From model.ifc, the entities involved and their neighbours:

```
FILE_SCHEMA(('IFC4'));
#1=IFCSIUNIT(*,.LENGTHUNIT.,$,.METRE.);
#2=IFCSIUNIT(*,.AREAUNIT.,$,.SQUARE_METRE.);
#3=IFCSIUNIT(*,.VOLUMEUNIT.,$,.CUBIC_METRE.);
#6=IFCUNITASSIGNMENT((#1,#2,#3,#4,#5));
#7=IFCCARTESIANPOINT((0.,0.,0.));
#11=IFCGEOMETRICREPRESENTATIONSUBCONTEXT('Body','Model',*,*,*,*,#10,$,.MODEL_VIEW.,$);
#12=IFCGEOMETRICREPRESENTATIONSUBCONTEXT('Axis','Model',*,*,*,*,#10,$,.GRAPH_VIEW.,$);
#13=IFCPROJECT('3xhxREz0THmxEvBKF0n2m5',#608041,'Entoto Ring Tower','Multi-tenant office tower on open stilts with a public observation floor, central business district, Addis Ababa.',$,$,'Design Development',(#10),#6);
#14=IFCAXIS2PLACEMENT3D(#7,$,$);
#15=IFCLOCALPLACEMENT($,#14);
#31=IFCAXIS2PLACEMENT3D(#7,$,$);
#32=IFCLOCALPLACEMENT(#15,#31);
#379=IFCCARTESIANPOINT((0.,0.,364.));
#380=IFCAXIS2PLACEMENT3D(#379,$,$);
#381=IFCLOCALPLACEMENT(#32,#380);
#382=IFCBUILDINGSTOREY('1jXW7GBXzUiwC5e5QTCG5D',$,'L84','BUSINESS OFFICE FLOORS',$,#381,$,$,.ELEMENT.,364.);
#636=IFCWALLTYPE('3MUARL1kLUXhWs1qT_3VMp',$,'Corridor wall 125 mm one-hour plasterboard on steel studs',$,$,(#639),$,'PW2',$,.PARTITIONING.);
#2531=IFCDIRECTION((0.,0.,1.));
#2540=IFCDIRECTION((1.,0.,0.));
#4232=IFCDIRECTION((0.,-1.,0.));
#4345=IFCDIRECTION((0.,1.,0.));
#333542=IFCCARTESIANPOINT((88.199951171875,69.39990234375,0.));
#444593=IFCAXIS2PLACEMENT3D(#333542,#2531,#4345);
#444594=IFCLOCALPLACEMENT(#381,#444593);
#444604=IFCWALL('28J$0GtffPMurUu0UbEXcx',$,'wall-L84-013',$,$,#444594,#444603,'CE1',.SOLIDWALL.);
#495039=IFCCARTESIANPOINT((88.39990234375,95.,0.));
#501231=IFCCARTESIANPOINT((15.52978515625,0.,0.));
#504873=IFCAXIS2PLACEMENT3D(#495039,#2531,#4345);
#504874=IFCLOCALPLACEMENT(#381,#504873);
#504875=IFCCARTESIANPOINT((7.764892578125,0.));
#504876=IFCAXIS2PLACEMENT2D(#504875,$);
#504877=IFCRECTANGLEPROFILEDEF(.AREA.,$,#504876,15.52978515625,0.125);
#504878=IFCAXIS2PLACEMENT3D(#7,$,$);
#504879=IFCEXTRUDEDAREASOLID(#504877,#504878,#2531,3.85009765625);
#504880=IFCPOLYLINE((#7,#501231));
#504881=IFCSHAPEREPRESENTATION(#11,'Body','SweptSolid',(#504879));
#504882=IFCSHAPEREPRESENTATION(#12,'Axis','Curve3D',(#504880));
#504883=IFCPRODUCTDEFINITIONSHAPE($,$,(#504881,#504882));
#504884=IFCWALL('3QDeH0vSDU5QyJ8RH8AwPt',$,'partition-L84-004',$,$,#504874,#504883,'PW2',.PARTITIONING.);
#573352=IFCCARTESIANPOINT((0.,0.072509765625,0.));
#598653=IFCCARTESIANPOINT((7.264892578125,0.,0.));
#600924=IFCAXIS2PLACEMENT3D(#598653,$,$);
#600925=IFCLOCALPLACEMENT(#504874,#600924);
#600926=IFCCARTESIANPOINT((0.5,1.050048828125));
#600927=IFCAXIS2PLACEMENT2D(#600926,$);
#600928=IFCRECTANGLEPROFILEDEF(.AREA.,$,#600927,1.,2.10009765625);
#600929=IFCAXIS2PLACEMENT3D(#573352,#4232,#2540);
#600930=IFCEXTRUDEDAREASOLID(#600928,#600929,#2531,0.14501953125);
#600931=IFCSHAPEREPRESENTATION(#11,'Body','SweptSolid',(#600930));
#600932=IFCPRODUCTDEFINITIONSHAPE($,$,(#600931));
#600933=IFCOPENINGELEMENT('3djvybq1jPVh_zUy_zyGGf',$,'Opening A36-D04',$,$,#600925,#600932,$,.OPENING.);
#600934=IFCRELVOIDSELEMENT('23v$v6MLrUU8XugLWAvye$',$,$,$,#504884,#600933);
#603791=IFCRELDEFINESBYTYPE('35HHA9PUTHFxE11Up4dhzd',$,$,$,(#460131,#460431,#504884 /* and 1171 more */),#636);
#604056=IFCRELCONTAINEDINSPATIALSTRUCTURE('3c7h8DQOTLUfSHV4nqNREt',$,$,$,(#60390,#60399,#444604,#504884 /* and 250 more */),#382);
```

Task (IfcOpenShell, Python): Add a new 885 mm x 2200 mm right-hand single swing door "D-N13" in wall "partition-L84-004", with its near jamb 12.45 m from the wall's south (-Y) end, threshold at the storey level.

```python
import numpy as np
import ifcopenshell
import ifcopenshell.api.feature
import ifcopenshell.api.geometry
import ifcopenshell.api.root
import ifcopenshell.api.spatial
import ifcopenshell.geom
import ifcopenshell.util.element
import ifcopenshell.util.placement
import ifcopenshell.util.representation
import ifcopenshell.util.shape
import ifcopenshell.util.unit

model = ifcopenshell.open("model.ifc")
unit_scale = ifcopenshell.util.unit.calculate_unit_scale(model)
settings = ifcopenshell.geom.settings()


def volume(element):
    """Net volume in cubic metres, openings subtracted."""
    shape = ifcopenshell.geom.create_shape(settings, element)
    return ifcopenshell.util.shape.get_volume(shape.geometry)


wall = model.by_guid("3QDeH0vSDU5QyJ8RH8AwPt")
storey = ifcopenshell.util.element.get_container(wall, ifc_class="IfcBuildingStorey")
context = ifcopenshell.util.representation.get_context(model, "Model", "Body", "MODEL_VIEW")
before = volume(wall)

width, height, from_end, sill = 0.885, 2.2, 12.45, 0.0  # metres

# The wall runs along its own X axis, and the end named is its -X end.
wall_shape = ifcopenshell.geom.create_shape(settings, wall)
x, y, z = ifcopenshell.util.shape.get_vertices(wall_shape.geometry).T
start = x.min() + from_end
face, thickness = float(y.min()), float(y.max() - y.min())
wall_matrix = ifcopenshell.util.placement.get_local_placement(wall.ObjectPlacement)
level = ifcopenshell.util.placement.get_local_placement(storey.ObjectPlacement)[2, 3]


def in_wall(x, y):
    """Placement at x, y metres in the wall's axes, at sill height."""
    matrix = wall_matrix.copy()
    matrix[:, 3] = wall_matrix @ np.array([x / unit_scale, y / unit_scale, 0.0, 1.0])
    matrix[2, 3] = level + sill / unit_scale
    return matrix


# Opening: a box that overshoots both wall faces by 50 mm.
opening = ifcopenshell.api.root.create_entity(model, ifc_class="IfcOpeningElement", predefined_type="OPENING")
box = ifcopenshell.api.geometry.add_wall_representation(
    model, context=context, length=width, height=height, thickness=thickness + 0.1
)
ifcopenshell.api.geometry.assign_representation(model, product=opening, representation=box)
ifcopenshell.api.geometry.edit_object_placement(model, product=opening, matrix=in_wall(start, face - 0.05), is_si=False)
ifcopenshell.api.feature.add_feature(model, feature=opening, element=wall)

door = ifcopenshell.api.root.create_entity(model, ifc_class="IfcDoor", name="D-N13", predefined_type="DOOR")
door.OverallWidth, door.OverallHeight = width / unit_scale, height / unit_scale
door.OperationType = "SINGLE_SWING_RIGHT"
body = ifcopenshell.api.geometry.add_door_representation(
    model,
    context=context,
    overall_width=door.OverallWidth,
    overall_height=door.OverallHeight,
    operation_type="SINGLE_SWING_RIGHT",
    lining_properties={"LiningDepth": thickness / unit_scale, "ThresholdDepth": thickness / unit_scale},
)
ifcopenshell.api.geometry.assign_representation(model, product=door, representation=body)
ifcopenshell.api.spatial.assign_container(model, products=[door], relating_structure=storey)
ifcopenshell.api.feature.add_filling(model, opening=opening, element=door)

# The lining spans the wall, so the door starts at the wall face.
ifcopenshell.api.geometry.edit_object_placement(model, product=door, matrix=in_wall(start, face), is_si=False)

after = volume(wall)

print(f"wall volume {before:.3f} -> {after:.3f} m3")

model.write("model_v2.ifc")
```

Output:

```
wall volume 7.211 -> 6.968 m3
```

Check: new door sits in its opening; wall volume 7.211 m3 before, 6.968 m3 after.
